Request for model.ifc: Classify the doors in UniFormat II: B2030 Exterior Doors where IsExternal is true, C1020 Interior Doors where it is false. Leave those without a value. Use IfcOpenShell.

First a look at what the model holds.

```python
import ifcopenshell
import ifcopenshell.util.element

model = ifcopenshell.open("model.ifc")
print(model.schema)
print("classifications:", [c.Name for c in model.by_type("IfcClassification")])
values = [ifcopenshell.util.element.get_pset(e, "Pset_DoorCommon", "IsExternal") for e in model.by_type("IfcDoor")]
for value in (True, False, None):
    print("IsExternal", value, values.count(value))
```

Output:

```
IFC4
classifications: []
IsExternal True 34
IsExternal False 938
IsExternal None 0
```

```python
import ifcopenshell
import ifcopenshell.api.classification
import ifcopenshell.util.element

model = ifcopenshell.open("model.ifc")

system = ifcopenshell.api.classification.add_classification(model, classification="UniFormat II")

doors = model.by_type("IfcDoor")
external = {e: ifcopenshell.util.element.get_pset(e, "Pset_DoorCommon", "IsExternal") for e in doors}
for flag, code, name in ((True, "B2030", "Exterior Doors"), (False, "C1020", "Interior Doors")):
    products = [e for e in doors if external[e] is flag]
    ifcopenshell.api.classification.add_reference(
        model, products=products, classification=system, identification=code, name=name
    )
    print(code, len(products))

model.write("model_rev.ifc")
```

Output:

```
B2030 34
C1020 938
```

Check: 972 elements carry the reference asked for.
